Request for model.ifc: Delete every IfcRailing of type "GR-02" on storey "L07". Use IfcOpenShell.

First a look at what the model holds.

```python
import ifcopenshell
import ifcopenshell.util.element

model = ifcopenshell.open("model.ifc")
print(model.schema)
storey = next(s for s in model.by_type("IfcBuildingStorey") if s.Name == "L07")
railings = [e for e in ifcopenshell.util.element.get_decomposition(storey) if e.is_a("IfcRailing")]
seen = {}
for e in railings:
    element_type = ifcopenshell.util.element.get_type(e)
    name = element_type.Name if element_type not in (None, e) else None
    seen[name] = seen.get(name, 0) + 1
for name, count in sorted(seen.items(), key=str):
    print(count, "x", name)
```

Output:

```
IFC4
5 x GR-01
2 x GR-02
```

```python
import ifcopenshell
import ifcopenshell.api.root
import ifcopenshell.util.element

model = ifcopenshell.open("model.ifc")

storey = next(s for s in model.by_type("IfcBuildingStorey") if s.Name == "L07")
railings = [e for e in ifcopenshell.util.element.get_decomposition(storey) if e.is_a("IfcRailing")]
targets = [e for e in railings if (t := ifcopenshell.util.element.get_type(e)) not in (None, e) and t.Name == "GR-02"]

for e in targets:
    ifcopenshell.api.root.remove_product(model, product=e)
print(len(targets), "removed")

model.write("model_v2.ifc")
```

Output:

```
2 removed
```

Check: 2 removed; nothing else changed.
